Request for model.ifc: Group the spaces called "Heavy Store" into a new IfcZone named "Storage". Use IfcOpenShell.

First a look at what the model holds.

```python
import ifcopenshell

model = ifcopenshell.open("model.ifc")
print(model.schema)
seen = {}
for space in model.by_type("IfcSpace"):
    seen[space.LongName] = seen.get(space.LongName, 0) + 1
for name, count in sorted(seen.items(), key=str):
    print(count, "x", name)
print("zones:", [z.Name for z in model.by_type("IfcZone")][:20])
```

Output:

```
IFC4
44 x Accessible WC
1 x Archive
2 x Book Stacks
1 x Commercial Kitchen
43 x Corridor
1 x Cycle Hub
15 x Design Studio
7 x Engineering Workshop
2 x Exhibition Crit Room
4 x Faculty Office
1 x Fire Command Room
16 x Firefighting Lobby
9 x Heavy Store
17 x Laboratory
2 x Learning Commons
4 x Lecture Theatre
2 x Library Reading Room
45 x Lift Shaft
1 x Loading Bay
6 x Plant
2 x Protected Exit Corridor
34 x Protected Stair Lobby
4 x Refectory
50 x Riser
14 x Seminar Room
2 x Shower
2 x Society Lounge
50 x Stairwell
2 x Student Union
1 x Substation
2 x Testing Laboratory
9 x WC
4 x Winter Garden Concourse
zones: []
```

```python
import ifcopenshell
import ifcopenshell.api.group
import ifcopenshell.api.root

model = ifcopenshell.open("model.ifc")

names = {"Heavy Store"}
spaces = [s for s in model.by_type("IfcSpace") if s.LongName in names]

zone = ifcopenshell.api.root.create_entity(model, ifc_class="IfcZone", name="Storage")
ifcopenshell.api.group.assign_group(model, products=spaces, group=zone)
print(len(spaces), "spaces in", zone.Name)

model.write("model_updated.ifc")
```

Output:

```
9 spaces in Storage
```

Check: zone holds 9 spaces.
